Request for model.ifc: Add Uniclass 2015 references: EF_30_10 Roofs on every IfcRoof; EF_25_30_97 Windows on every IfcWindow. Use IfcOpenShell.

First a look at what the model holds.

```python
import ifcopenshell

model = ifcopenshell.open("model.ifc")
print(model.schema)
print("classifications:", [c.Name for c in model.by_type("IfcClassification")])
for ifc_class in ("IfcDoor", "IfcRoof", "IfcStair", "IfcWall", "IfcWindow"):
    print(ifc_class, len(model.by_type(ifc_class)))
```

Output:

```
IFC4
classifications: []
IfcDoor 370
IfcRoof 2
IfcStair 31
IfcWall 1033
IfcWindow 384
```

```python
import ifcopenshell
import ifcopenshell.api.classification

model = ifcopenshell.open("model.ifc")

system = ifcopenshell.api.classification.add_classification(model, classification="Uniclass 2015")

codes = {
    "IfcRoof": ("EF_30_10", "Roofs"),
    "IfcWindow": ("EF_25_30_97", "Windows"),
}
for ifc_class, (code, name) in codes.items():
    products = model.by_type(ifc_class)
    ifcopenshell.api.classification.add_reference(
        model, products=products, classification=system, identification=code, name=name
    )
    print(code, len(products))

model.write("model_edited.ifc")
```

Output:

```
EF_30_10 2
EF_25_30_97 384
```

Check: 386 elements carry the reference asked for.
